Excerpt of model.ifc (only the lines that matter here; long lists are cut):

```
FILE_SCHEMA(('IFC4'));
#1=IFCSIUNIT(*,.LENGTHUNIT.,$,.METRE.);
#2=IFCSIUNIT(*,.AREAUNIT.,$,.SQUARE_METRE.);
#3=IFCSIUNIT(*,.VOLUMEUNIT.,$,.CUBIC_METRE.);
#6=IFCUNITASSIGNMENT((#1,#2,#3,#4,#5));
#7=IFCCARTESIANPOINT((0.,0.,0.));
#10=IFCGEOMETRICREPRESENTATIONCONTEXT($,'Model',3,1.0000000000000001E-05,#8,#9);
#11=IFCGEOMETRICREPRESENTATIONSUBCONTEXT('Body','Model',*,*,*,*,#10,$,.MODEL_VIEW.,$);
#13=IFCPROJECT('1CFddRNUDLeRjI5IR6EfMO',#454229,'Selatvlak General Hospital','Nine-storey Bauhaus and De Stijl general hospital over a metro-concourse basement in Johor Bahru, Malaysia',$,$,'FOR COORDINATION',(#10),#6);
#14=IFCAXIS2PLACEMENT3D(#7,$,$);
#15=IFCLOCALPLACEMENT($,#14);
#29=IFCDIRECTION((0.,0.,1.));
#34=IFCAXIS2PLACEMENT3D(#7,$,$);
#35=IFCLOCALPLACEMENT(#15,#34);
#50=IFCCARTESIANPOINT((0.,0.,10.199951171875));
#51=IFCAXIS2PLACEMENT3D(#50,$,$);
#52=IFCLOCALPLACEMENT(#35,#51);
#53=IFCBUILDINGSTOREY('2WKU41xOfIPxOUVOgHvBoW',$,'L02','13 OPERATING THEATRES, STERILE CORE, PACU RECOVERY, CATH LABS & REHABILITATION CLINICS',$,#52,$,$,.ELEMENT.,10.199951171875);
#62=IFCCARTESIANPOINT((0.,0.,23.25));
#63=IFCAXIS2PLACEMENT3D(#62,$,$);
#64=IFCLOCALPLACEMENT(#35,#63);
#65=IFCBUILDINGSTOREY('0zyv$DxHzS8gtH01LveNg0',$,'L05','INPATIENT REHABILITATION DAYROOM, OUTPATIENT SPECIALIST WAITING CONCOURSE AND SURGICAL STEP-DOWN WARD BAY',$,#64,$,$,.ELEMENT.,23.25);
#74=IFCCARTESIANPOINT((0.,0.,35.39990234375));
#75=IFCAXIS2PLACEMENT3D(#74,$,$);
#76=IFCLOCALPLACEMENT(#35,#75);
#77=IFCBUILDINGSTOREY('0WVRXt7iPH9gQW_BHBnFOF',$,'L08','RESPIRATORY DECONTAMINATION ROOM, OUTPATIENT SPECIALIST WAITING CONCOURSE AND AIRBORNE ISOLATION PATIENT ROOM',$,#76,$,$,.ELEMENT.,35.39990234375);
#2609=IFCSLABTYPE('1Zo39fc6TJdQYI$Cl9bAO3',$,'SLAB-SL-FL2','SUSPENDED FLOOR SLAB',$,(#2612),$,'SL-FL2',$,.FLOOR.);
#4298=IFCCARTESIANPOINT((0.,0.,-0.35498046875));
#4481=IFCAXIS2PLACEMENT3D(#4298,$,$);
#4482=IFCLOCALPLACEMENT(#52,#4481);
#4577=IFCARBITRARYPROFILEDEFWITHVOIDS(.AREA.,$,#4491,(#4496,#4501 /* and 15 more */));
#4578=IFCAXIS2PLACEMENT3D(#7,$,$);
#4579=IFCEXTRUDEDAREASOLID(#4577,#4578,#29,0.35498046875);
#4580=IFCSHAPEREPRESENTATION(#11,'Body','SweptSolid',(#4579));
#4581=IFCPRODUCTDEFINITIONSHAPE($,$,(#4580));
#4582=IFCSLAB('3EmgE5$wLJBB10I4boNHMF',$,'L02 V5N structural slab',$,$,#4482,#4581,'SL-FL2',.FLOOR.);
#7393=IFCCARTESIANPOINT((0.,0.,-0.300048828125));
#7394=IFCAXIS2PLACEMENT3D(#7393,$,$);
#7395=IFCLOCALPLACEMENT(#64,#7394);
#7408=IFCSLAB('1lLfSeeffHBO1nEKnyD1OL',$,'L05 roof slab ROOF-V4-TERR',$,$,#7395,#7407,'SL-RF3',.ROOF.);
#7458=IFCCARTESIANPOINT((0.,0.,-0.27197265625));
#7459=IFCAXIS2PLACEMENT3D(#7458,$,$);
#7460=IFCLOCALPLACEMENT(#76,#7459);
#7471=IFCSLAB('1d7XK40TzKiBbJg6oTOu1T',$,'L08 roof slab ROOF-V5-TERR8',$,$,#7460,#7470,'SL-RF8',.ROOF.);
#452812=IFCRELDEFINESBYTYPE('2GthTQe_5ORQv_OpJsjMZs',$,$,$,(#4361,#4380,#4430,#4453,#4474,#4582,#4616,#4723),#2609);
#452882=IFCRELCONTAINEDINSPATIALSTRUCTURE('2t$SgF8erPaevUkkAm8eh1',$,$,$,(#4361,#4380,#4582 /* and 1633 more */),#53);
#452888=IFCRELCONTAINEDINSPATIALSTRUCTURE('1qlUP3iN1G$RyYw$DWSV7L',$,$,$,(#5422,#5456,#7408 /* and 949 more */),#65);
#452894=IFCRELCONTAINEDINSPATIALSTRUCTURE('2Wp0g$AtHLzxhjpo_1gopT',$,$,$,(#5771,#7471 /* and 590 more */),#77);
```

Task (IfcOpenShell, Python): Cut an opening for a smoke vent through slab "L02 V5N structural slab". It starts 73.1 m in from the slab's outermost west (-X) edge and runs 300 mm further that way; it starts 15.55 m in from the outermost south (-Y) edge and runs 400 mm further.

```python
import numpy as np
import ifcopenshell
import ifcopenshell.api.feature
import ifcopenshell.api.geometry
import ifcopenshell.api.root
import ifcopenshell.geom
import ifcopenshell.util.placement
import ifcopenshell.util.representation
import ifcopenshell.util.shape
import ifcopenshell.util.unit

model = ifcopenshell.open("model.ifc")
unit_scale = ifcopenshell.util.unit.calculate_unit_scale(model)
settings = ifcopenshell.geom.settings()


def volume(element):
    """Net volume in cubic metres, openings subtracted."""
    shape = ifcopenshell.geom.create_shape(settings, element)
    return ifcopenshell.util.shape.get_volume(shape.geometry)


slab = model.by_guid("3EmgE5$wLJBB10I4boNHMF")
before = volume(slab)

# Extent in the slab's own axes, in metres. The edges named are its -X and -Y sides.
slab_shape = ifcopenshell.geom.create_shape(settings, slab)
vertices = ifcopenshell.util.shape.get_vertices(slab_shape.geometry)
x_min, y_min, bottom = vertices.min(axis=0)
top = vertices[:, 2].max()

opening = ifcopenshell.api.root.create_entity(model, ifc_class="IfcOpeningElement", name="Smoke vent opening", predefined_type="OPENING")
context = ifcopenshell.util.representation.get_context(model, "Model", "Body", "MODEL_VIEW")
width, depth = 0.3, 0.4
outline = [(0.0, 0.0), (width, 0.0), (width, depth), (0.0, depth), (0.0, 0.0)]
# Overshoot both faces by 50 mm so the cut is clean.
shape = ifcopenshell.api.geometry.add_slab_representation(
    model, context=context, depth=top - bottom + 0.1, polyline=outline
)
ifcopenshell.api.geometry.assign_representation(model, product=opening, representation=shape)

matrix = ifcopenshell.util.placement.get_local_placement(slab.ObjectPlacement)
matrix[:, 3] = matrix @ np.append(np.array([x_min + 73.1, y_min + 15.55, bottom - 0.05]) / unit_scale, 1.0)
ifcopenshell.api.geometry.edit_object_placement(model, product=opening, matrix=matrix, is_si=False)
ifcopenshell.api.feature.add_feature(model, feature=opening, element=slab)

after = volume(slab)

print(f"slab volume {before:.3f} -> {after:.3f} m3")

model.write("model-out.ifc")
```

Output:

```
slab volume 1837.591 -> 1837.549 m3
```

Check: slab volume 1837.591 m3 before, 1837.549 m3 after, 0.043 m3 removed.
